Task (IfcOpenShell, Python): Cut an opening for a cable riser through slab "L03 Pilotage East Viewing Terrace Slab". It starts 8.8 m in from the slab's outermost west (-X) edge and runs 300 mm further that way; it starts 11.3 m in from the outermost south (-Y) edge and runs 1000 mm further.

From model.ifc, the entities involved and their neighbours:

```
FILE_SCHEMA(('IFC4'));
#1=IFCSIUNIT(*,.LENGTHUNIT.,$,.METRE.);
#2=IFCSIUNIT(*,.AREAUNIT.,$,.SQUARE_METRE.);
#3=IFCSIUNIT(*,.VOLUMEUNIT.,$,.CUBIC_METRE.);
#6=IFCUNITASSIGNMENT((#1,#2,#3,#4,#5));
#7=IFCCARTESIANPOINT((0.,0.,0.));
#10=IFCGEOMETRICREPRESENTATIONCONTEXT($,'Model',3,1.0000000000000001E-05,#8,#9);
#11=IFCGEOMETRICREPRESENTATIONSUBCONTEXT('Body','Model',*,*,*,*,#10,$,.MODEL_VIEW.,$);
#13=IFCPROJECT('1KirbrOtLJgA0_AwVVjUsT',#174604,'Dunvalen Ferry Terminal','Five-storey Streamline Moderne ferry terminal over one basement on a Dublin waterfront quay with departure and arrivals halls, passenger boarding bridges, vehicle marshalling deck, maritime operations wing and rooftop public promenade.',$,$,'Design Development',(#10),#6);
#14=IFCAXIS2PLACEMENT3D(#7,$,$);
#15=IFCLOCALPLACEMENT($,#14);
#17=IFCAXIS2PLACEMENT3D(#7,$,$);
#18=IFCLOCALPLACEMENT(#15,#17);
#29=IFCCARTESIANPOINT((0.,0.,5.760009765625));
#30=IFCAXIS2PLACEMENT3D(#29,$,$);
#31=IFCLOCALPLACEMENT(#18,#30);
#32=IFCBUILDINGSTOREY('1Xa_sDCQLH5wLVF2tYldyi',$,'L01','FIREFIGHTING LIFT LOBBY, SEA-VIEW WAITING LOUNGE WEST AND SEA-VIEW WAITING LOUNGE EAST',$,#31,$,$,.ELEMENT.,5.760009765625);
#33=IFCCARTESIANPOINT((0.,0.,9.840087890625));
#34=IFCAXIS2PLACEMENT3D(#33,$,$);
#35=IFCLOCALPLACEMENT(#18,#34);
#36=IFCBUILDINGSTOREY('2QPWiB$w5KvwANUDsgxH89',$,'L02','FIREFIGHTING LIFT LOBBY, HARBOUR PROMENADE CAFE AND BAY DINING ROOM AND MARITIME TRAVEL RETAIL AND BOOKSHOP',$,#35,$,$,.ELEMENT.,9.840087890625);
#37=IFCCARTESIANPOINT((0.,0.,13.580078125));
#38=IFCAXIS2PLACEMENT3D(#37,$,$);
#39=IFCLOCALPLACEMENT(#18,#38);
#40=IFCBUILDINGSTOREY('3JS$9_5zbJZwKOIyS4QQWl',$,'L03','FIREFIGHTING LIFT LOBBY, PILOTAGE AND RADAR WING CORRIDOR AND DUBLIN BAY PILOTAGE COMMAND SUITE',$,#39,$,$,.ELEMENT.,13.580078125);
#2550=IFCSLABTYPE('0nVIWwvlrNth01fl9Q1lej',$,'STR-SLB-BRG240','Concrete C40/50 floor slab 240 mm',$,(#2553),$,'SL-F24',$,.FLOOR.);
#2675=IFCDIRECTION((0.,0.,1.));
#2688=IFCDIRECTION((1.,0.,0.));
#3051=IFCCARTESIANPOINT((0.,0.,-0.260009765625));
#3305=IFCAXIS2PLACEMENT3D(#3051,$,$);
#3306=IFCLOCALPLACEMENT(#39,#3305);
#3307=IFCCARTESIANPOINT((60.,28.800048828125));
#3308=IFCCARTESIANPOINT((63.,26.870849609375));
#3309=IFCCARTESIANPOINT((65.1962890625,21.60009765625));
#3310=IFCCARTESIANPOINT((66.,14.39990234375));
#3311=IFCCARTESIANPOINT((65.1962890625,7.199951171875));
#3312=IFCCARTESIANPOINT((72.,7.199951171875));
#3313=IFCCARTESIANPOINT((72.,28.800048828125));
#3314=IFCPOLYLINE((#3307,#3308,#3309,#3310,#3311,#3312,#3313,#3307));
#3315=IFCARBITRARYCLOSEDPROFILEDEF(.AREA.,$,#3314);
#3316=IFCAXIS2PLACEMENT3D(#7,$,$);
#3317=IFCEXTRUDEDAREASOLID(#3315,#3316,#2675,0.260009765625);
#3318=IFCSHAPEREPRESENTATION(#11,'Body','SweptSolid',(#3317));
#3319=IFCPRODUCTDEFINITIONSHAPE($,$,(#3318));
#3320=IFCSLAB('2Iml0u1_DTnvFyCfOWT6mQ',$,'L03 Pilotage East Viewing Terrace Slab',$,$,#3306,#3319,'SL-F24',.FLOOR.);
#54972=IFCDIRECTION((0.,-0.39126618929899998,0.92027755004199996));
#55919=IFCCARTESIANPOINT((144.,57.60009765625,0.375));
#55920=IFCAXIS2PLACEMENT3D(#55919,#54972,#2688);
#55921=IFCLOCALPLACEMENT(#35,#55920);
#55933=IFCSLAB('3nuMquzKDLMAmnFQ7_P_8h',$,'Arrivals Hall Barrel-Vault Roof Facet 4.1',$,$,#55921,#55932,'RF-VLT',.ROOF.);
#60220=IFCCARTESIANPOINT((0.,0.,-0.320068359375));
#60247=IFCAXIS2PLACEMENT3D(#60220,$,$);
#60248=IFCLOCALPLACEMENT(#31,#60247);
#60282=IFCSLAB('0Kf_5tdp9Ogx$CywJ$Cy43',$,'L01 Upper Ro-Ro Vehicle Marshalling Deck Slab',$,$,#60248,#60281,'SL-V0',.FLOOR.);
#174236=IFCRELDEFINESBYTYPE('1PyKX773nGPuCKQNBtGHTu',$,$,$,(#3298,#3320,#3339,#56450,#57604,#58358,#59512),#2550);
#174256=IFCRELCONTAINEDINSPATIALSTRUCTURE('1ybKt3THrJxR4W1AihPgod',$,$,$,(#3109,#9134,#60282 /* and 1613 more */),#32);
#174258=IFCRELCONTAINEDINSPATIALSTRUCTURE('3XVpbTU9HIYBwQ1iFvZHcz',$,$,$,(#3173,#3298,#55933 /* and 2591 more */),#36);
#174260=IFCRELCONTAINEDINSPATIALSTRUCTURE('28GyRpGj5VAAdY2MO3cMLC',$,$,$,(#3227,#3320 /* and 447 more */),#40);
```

```python
import numpy as np
import ifcopenshell
import ifcopenshell.api.feature
import ifcopenshell.api.geometry
import ifcopenshell.api.root
import ifcopenshell.geom
import ifcopenshell.util.placement
import ifcopenshell.util.representation
import ifcopenshell.util.shape
import ifcopenshell.util.unit

model = ifcopenshell.open("model.ifc")
unit_scale = ifcopenshell.util.unit.calculate_unit_scale(model)
settings = ifcopenshell.geom.settings()


def volume(element):
    """Net volume in cubic metres, openings subtracted."""
    shape = ifcopenshell.geom.create_shape(settings, element)
    return ifcopenshell.util.shape.get_volume(shape.geometry)


slab = model.by_guid("2Iml0u1_DTnvFyCfOWT6mQ")
before = volume(slab)

# Extent in the slab's own axes, in metres. The edges named are its -X and -Y sides.
slab_shape = ifcopenshell.geom.create_shape(settings, slab)
vertices = ifcopenshell.util.shape.get_vertices(slab_shape.geometry)
x_min, y_min, bottom = vertices.min(axis=0)
top = vertices[:, 2].max()

opening = ifcopenshell.api.root.create_entity(model, ifc_class="IfcOpeningElement", name="Cable riser opening", predefined_type="OPENING")
context = ifcopenshell.util.representation.get_context(model, "Model", "Body", "MODEL_VIEW")
width, depth = 0.3, 1
outline = [(0.0, 0.0), (width, 0.0), (width, depth), (0.0, depth), (0.0, 0.0)]
# Overshoot both faces by 50 mm so the cut is clean.
shape = ifcopenshell.api.geometry.add_slab_representation(
    model, context=context, depth=top - bottom + 0.1, polyline=outline
)
ifcopenshell.api.geometry.assign_representation(model, product=opening, representation=shape)

matrix = ifcopenshell.util.placement.get_local_placement(slab.ObjectPlacement)
matrix[:, 3] = matrix @ np.append(np.array([x_min + 8.8, y_min + 11.3, bottom - 0.05]) / unit_scale, 1.0)
ifcopenshell.api.geometry.edit_object_placement(model, product=opening, matrix=matrix, is_si=False)
ifcopenshell.api.feature.add_feature(model, feature=opening, element=slab)

after = volume(slab)

print(f"slab volume {before:.3f} -> {after:.3f} m3")

model.write("model_edited.ifc")
```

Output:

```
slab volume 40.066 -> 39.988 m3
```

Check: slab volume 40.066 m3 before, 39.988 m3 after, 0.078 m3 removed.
